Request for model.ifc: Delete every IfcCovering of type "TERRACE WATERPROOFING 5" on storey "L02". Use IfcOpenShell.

First a look at what the model holds.

```python
import ifcopenshell
import ifcopenshell.util.element

model = ifcopenshell.open("model.ifc")
print(model.schema)
storey = next(s for s in model.by_type("IfcBuildingStorey") if s.Name == "L02")
coverings = [e for e in ifcopenshell.util.element.get_decomposition(storey) if e.is_a("IfcCovering")]
seen = {}
for e in coverings:
    element_type = ifcopenshell.util.element.get_type(e)
    name = element_type.Name if element_type not in (None, e) else None
    seen[name] = seen.get(name, 0) + 1
for name, count in sorted(seen.items(), key=str):
    print(count, "x", name)
```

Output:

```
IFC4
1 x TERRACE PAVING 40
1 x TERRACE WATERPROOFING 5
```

```python
import ifcopenshell
import ifcopenshell.api.root
import ifcopenshell.util.element

model = ifcopenshell.open("model.ifc")

storey = next(s for s in model.by_type("IfcBuildingStorey") if s.Name == "L02")
coverings = [e for e in ifcopenshell.util.element.get_decomposition(storey) if e.is_a("IfcCovering")]
targets = [e for e in coverings if (t := ifcopenshell.util.element.get_type(e)) not in (None, e) and t.Name == "TERRACE WATERPROOFING 5"]

for e in targets:
    ifcopenshell.api.root.remove_product(model, product=e)
print(len(targets), "removed")

model.write("model_v2.ifc")
```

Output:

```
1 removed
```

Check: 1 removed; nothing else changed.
